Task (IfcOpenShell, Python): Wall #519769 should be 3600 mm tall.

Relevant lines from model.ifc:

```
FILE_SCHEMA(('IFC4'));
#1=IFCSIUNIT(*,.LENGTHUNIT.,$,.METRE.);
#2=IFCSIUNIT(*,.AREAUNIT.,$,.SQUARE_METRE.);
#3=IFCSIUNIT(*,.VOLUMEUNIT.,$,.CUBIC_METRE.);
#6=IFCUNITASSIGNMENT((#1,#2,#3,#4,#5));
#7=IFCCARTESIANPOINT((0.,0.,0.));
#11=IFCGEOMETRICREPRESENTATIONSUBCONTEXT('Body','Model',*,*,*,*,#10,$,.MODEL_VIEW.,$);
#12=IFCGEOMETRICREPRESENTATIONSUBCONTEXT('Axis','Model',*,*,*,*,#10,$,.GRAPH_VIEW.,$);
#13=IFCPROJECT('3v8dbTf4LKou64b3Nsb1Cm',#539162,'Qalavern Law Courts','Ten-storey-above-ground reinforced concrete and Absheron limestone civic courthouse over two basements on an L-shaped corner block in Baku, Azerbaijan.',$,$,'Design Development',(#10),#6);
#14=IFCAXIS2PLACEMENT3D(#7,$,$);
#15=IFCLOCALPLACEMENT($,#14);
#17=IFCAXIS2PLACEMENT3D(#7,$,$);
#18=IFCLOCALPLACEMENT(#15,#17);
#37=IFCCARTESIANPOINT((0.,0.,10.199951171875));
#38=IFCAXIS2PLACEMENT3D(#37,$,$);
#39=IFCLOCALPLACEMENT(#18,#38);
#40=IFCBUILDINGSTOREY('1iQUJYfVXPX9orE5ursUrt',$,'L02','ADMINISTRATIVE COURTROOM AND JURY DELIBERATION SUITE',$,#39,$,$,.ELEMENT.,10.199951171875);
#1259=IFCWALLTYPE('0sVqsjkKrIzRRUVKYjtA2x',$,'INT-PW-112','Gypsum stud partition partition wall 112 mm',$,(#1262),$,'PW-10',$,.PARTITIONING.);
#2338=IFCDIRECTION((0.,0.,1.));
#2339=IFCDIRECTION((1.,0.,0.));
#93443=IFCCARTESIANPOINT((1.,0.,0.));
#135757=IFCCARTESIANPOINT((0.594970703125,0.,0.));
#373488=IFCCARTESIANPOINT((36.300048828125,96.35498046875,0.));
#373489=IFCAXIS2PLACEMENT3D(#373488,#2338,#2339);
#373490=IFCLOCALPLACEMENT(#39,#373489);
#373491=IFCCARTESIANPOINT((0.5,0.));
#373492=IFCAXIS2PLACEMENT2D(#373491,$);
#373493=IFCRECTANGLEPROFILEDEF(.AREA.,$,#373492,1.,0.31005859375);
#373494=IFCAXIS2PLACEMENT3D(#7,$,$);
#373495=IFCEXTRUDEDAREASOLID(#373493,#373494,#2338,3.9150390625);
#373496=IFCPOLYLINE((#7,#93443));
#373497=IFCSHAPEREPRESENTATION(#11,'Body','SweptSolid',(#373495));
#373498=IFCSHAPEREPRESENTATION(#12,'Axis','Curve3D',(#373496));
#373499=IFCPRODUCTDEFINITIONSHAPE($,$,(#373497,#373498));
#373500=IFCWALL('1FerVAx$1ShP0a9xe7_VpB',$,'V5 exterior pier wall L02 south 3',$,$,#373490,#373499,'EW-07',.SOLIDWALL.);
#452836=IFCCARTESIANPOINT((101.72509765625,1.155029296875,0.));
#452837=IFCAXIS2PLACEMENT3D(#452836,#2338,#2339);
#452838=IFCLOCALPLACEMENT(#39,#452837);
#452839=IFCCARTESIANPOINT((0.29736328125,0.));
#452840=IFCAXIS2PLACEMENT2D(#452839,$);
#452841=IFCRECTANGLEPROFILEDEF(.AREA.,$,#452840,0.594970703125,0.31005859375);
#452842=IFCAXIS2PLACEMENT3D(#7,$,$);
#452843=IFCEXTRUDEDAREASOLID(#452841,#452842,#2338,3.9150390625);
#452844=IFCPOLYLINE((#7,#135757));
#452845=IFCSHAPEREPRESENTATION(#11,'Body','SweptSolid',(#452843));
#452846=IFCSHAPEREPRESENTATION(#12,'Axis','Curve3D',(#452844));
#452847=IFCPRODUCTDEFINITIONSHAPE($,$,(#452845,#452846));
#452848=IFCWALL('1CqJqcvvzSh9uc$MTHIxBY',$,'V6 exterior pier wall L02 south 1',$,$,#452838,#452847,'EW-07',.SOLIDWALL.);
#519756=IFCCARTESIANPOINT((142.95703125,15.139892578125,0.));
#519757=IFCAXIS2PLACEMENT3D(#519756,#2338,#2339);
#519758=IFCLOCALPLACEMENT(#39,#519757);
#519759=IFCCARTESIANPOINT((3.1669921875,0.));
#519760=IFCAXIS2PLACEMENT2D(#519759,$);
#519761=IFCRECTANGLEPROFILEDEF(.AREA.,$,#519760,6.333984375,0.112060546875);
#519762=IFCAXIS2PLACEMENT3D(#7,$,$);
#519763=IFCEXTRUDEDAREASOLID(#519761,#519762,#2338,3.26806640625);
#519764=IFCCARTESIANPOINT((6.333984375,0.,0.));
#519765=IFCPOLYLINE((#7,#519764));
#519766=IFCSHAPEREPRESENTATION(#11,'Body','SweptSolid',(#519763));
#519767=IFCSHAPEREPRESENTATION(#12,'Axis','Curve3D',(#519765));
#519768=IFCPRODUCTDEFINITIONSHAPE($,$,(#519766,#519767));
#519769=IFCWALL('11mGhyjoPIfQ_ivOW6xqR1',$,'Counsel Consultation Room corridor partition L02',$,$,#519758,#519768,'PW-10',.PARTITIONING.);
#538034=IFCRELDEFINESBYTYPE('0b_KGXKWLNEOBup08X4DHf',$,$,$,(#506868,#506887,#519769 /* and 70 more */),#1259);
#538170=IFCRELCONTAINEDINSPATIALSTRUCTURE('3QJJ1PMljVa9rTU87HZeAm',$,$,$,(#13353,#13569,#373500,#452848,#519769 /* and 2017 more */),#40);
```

```python
import ifcopenshell
import ifcopenshell.geom
import ifcopenshell.util.representation
import ifcopenshell.util.shape
import ifcopenshell.util.unit

model = ifcopenshell.open("model.ifc")
unit_scale = ifcopenshell.util.unit.calculate_unit_scale(model)
settings = ifcopenshell.geom.settings()


def volume(element):
    """Net volume in cubic metres, openings subtracted."""
    shape = ifcopenshell.geom.create_shape(settings, element)
    return ifcopenshell.util.shape.get_volume(shape.geometry)


wall = model.by_guid("11mGhyjoPIfQ_ivOW6xqR1")
before = volume(wall)

body = ifcopenshell.util.representation.get_representation(wall, "Model", "Body")
solid = body.Items[0]
old_height = solid.Depth
solid.Depth = 3.6 / unit_scale
after = volume(wall)

print(f"height {old_height:g} -> {solid.Depth:g}, volume {before:.3f} -> {after:.3f} m3")

model.write("model_v2.ifc")
```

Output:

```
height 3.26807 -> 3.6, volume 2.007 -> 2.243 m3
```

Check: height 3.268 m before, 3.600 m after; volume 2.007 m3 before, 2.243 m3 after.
